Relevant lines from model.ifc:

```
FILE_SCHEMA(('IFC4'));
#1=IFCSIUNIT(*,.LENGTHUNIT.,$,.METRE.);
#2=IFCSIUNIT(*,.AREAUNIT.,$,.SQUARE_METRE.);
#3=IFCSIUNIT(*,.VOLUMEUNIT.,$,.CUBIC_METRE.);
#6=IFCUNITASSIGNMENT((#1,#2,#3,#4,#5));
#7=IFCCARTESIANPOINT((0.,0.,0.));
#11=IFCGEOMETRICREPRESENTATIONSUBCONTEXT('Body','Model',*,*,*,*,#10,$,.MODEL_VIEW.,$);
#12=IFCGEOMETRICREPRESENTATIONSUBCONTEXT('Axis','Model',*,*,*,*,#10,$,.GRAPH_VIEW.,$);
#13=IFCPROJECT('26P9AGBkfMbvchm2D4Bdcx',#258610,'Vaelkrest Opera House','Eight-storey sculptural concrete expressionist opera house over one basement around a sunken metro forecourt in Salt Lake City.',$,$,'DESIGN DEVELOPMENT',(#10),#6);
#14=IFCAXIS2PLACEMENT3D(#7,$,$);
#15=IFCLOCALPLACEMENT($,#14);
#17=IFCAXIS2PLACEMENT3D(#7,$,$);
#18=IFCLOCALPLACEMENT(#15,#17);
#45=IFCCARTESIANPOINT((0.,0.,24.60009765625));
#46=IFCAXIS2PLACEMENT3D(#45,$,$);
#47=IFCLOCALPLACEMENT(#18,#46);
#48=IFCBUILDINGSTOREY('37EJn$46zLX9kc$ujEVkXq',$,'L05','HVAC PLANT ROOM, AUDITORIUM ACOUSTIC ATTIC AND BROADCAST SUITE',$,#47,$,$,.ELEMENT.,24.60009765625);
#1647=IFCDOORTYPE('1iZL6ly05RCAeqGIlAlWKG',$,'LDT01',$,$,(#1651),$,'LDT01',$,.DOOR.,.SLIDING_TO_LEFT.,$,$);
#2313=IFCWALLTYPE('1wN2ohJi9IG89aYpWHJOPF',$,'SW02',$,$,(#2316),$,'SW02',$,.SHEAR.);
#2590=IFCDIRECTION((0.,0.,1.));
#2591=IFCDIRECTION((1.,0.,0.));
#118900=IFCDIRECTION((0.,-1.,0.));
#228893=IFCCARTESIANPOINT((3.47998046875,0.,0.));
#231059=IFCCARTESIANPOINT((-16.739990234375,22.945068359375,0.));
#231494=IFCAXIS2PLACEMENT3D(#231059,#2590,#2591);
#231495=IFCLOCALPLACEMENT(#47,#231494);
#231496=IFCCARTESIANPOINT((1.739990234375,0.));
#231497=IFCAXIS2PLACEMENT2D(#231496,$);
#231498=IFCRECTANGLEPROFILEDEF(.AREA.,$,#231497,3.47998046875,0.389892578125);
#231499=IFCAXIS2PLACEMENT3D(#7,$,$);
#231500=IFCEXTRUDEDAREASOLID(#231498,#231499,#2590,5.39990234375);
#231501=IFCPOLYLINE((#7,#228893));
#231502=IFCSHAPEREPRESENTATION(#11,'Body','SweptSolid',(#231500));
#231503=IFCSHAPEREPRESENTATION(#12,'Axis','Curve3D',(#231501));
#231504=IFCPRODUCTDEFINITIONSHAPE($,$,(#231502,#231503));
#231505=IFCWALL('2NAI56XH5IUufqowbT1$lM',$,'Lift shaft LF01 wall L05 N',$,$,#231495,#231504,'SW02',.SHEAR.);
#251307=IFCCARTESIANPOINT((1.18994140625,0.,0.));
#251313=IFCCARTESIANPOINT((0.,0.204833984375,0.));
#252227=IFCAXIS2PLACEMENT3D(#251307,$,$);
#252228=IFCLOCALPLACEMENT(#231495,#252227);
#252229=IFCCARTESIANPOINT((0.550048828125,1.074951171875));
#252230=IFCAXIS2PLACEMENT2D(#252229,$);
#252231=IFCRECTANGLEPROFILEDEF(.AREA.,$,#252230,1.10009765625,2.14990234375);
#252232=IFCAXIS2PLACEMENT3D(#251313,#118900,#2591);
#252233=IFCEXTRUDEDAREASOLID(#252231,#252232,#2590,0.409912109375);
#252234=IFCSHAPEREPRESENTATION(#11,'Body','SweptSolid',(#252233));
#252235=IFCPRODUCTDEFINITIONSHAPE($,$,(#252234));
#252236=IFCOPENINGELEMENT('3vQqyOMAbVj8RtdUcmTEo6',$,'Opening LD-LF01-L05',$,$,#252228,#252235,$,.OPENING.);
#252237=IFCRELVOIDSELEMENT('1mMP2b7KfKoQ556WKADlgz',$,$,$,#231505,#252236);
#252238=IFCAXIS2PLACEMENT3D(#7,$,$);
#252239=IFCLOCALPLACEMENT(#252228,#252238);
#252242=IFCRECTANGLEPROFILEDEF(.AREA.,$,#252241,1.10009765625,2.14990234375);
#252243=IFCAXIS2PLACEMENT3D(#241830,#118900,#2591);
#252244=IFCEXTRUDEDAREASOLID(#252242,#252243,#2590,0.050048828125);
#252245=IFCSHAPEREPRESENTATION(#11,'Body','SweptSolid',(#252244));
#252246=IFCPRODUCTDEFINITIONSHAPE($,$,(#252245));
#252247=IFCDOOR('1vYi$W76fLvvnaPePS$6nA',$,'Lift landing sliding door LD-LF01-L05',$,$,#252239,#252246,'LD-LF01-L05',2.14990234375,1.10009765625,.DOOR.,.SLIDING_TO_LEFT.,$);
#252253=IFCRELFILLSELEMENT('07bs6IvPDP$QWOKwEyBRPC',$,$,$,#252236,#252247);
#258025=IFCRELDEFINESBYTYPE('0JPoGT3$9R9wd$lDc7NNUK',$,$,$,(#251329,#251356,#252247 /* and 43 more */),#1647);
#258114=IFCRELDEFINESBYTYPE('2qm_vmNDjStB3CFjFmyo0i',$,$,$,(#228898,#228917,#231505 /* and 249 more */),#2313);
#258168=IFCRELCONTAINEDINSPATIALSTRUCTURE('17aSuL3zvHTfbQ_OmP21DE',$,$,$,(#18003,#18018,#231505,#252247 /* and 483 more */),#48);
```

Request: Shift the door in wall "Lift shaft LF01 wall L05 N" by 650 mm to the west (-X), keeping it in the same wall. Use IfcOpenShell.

```python
import ifcopenshell
import ifcopenshell.api.geometry
import ifcopenshell.util.placement

model = ifcopenshell.open("model.ifc")

door = model.by_guid("1vYi$W76fLvvnaPePS$6nA")
opening = door.FillsVoids[0].RelatingOpeningElement
wall = opening.VoidsElements[0].RelatingBuildingElement

wall_matrix = ifcopenshell.util.placement.get_local_placement(wall.ObjectPlacement)
shift = wall_matrix[:3, 0] * -0.65
before = ifcopenshell.util.placement.get_local_placement(door.ObjectPlacement)[:3, 3].copy()

# The door is placed relative to its opening, so it follows when the opening moves.
matrix = ifcopenshell.util.placement.get_local_placement(opening.ObjectPlacement)
matrix[:3, 3] += shift
ifcopenshell.api.geometry.edit_object_placement(
    model, product=opening, matrix=matrix, is_si=False, should_transform_children=True
)

after = ifcopenshell.util.placement.get_local_placement(door.ObjectPlacement)[:3, 3]
print("door moved by", (after - before).round(3) + 0.0)

model.write("model-out.ifc")
```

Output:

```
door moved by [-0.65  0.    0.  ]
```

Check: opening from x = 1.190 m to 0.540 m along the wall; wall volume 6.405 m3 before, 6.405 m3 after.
